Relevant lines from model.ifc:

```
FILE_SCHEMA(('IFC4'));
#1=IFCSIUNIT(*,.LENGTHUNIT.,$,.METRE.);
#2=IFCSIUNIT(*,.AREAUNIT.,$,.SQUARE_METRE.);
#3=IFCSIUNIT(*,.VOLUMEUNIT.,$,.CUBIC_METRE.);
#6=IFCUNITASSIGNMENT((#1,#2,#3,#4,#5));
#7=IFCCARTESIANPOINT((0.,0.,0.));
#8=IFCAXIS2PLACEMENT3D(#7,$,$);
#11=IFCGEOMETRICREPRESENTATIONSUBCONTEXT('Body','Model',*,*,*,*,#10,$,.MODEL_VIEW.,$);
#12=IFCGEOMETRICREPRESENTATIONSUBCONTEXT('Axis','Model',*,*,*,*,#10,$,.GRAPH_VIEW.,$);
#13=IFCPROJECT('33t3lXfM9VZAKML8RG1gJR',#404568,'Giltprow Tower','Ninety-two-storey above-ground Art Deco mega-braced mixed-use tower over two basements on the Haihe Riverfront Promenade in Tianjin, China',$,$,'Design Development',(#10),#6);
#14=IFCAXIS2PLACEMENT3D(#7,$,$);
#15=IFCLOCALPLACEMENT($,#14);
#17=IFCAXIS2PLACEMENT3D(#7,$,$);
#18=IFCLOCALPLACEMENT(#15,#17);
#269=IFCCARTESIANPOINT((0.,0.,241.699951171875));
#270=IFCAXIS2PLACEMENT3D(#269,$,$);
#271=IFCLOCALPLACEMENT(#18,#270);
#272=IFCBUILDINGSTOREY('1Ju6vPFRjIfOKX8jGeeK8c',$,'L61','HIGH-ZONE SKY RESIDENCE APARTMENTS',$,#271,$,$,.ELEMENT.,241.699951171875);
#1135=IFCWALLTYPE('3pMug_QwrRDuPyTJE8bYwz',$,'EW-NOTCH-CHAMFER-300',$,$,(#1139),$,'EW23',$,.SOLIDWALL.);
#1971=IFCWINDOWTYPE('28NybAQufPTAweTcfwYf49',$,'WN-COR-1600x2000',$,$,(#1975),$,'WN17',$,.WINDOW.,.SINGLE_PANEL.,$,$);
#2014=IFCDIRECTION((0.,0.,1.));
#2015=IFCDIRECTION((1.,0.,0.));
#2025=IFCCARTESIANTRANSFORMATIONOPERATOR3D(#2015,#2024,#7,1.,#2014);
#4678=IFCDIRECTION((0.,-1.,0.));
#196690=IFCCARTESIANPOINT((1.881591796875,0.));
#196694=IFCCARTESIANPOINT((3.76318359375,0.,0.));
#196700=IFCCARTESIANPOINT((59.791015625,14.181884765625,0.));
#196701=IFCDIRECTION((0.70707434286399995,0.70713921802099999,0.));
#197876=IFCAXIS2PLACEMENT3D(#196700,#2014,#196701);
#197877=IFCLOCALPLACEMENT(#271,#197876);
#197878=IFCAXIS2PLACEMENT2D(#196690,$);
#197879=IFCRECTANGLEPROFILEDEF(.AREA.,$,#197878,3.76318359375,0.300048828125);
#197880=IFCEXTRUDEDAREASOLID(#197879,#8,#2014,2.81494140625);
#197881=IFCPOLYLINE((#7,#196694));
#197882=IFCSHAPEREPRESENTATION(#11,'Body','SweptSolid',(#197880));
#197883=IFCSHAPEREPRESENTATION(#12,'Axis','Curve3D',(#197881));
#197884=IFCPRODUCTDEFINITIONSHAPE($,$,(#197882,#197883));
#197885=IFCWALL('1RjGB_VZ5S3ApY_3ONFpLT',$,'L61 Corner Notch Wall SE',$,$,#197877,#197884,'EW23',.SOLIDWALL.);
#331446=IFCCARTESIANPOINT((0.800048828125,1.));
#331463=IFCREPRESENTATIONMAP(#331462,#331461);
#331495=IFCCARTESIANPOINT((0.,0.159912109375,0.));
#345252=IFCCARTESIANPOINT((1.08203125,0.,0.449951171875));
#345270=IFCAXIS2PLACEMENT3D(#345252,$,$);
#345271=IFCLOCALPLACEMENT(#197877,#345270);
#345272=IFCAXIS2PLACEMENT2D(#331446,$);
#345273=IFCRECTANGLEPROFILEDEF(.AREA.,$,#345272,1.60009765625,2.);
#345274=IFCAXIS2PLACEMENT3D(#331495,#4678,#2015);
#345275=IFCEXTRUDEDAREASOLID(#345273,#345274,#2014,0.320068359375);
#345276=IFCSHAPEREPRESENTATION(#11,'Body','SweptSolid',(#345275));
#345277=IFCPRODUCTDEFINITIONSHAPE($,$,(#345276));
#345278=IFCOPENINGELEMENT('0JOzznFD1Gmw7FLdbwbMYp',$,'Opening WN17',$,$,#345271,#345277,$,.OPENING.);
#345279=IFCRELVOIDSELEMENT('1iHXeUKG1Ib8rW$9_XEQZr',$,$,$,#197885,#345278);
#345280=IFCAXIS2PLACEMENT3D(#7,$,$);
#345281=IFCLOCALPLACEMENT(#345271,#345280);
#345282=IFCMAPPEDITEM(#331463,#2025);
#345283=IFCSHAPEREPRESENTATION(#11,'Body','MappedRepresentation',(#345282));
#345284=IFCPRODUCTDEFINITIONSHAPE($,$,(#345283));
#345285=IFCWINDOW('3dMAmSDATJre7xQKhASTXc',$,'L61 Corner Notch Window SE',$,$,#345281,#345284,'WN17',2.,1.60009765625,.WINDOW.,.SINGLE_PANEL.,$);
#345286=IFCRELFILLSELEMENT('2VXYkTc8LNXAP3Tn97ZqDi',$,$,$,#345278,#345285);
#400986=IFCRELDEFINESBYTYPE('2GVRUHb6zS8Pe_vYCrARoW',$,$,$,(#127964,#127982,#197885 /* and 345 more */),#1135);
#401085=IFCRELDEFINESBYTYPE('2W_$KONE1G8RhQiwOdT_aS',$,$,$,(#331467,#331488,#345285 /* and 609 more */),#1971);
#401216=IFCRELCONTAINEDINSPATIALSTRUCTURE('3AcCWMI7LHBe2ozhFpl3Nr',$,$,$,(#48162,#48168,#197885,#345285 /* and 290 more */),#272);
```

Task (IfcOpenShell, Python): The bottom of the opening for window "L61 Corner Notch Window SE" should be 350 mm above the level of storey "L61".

```python
import numpy as np
import ifcopenshell
import ifcopenshell.api.geometry
import ifcopenshell.geom
import ifcopenshell.util.element
import ifcopenshell.util.placement
import ifcopenshell.util.shape
import ifcopenshell.util.unit

model = ifcopenshell.open("model.ifc")
unit_scale = ifcopenshell.util.unit.calculate_unit_scale(model)

window = model.by_id(345285)
opening = window.FillsVoids[0].RelatingOpeningElement
storey = ifcopenshell.util.element.get_container(window, ifc_class="IfcBuildingStorey")
level = ifcopenshell.util.placement.get_local_placement(storey.ObjectPlacement)[2, 3]

# The opening's origin need not be at the sill, so measure its lowest point.
shape = ifcopenshell.geom.create_shape(ifcopenshell.geom.settings(), opening)
bottom = ifcopenshell.util.shape.get_shape_bottom_elevation(shape, shape.geometry) / unit_scale
dz = level + 0.35 / unit_scale - bottom

shift = np.array([0.0, 0.0, dz])
# The window is placed relative to its opening, so it follows when the opening moves.
matrix = ifcopenshell.util.placement.get_local_placement(opening.ObjectPlacement)
matrix[:3, 3] += shift
ifcopenshell.api.geometry.edit_object_placement(
    model, product=opening, matrix=matrix, is_si=False, should_transform_children=True
)

print(f"moved by {dz * unit_scale:+.3f} m")

model.write("model_rev.ifc")
```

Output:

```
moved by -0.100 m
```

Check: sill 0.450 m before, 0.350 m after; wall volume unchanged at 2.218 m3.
